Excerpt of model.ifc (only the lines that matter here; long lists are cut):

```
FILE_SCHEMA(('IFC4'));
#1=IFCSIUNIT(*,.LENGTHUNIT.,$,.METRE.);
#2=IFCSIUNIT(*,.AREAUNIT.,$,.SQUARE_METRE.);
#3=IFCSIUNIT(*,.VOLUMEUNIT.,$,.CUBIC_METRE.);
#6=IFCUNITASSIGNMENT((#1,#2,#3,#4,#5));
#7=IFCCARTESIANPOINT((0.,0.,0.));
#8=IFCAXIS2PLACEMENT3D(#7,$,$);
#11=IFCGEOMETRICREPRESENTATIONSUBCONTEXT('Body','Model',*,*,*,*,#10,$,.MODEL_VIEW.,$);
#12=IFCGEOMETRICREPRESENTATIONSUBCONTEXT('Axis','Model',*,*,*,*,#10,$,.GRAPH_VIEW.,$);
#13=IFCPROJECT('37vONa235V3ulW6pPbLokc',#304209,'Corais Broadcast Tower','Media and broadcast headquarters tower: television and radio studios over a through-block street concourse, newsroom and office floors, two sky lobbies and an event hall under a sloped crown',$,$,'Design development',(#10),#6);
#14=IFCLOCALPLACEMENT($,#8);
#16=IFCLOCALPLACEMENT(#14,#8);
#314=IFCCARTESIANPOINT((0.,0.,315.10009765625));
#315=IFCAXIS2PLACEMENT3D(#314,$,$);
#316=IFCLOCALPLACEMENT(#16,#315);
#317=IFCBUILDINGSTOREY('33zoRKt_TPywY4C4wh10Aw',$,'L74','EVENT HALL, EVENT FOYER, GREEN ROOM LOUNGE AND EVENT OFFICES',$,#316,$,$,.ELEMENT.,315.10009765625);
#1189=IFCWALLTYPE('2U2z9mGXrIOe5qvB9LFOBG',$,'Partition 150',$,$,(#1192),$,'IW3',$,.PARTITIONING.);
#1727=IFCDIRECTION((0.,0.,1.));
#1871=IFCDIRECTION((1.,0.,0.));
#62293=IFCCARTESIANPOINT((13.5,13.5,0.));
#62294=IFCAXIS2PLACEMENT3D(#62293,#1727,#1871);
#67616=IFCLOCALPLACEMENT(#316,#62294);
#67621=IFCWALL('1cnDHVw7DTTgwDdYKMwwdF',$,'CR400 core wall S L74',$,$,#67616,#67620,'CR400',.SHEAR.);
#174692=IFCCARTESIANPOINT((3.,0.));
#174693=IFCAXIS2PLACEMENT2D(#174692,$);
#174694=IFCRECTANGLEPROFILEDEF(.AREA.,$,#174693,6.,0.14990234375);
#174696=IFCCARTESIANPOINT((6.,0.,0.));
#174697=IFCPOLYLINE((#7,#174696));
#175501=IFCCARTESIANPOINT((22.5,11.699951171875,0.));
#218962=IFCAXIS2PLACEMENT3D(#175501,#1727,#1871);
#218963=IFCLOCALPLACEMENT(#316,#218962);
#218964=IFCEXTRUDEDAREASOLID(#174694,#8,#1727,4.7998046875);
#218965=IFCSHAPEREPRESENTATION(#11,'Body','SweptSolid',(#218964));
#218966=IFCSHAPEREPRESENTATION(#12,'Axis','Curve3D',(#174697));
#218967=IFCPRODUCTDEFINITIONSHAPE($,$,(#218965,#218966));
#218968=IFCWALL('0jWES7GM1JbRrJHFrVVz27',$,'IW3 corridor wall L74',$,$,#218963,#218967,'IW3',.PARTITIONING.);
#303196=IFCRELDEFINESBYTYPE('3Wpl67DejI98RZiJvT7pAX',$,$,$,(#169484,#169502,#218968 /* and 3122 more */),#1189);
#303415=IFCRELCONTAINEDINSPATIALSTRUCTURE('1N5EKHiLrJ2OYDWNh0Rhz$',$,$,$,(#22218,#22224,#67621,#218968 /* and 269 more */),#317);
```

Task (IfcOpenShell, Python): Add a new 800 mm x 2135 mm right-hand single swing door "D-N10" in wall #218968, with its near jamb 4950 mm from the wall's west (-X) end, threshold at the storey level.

```python
import numpy as np
import ifcopenshell
import ifcopenshell.api.feature
import ifcopenshell.api.geometry
import ifcopenshell.api.root
import ifcopenshell.api.spatial
import ifcopenshell.geom
import ifcopenshell.util.element
import ifcopenshell.util.placement
import ifcopenshell.util.representation
import ifcopenshell.util.shape
import ifcopenshell.util.unit

model = ifcopenshell.open("model.ifc")
unit_scale = ifcopenshell.util.unit.calculate_unit_scale(model)
settings = ifcopenshell.geom.settings()


def volume(element):
    """Net volume in cubic metres, openings subtracted."""
    shape = ifcopenshell.geom.create_shape(settings, element)
    return ifcopenshell.util.shape.get_volume(shape.geometry)


wall = model.by_guid("0jWES7GM1JbRrJHFrVVz27")
storey = ifcopenshell.util.element.get_container(wall, ifc_class="IfcBuildingStorey")
context = ifcopenshell.util.representation.get_context(model, "Model", "Body", "MODEL_VIEW")
before = volume(wall)

width, height, from_end, sill = 0.8, 2.135, 4.95, 0.0  # metres

# The wall runs along its own X axis, and the end named is its -X end.
wall_shape = ifcopenshell.geom.create_shape(settings, wall)
x, y, z = ifcopenshell.util.shape.get_vertices(wall_shape.geometry).T
start = x.min() + from_end
face, thickness = float(y.min()), float(y.max() - y.min())
wall_matrix = ifcopenshell.util.placement.get_local_placement(wall.ObjectPlacement)
level = ifcopenshell.util.placement.get_local_placement(storey.ObjectPlacement)[2, 3]


def in_wall(x, y):
    """Placement at x, y metres in the wall's axes, at sill height."""
    matrix = wall_matrix.copy()
    matrix[:, 3] = wall_matrix @ np.array([x / unit_scale, y / unit_scale, 0.0, 1.0])
    matrix[2, 3] = level + sill / unit_scale
    return matrix


# Opening: a box that overshoots both wall faces by 50 mm.
opening = ifcopenshell.api.root.create_entity(model, ifc_class="IfcOpeningElement", predefined_type="OPENING")
box = ifcopenshell.api.geometry.add_wall_representation(
    model, context=context, length=width, height=height, thickness=thickness + 0.1
)
ifcopenshell.api.geometry.assign_representation(model, product=opening, representation=box)
ifcopenshell.api.geometry.edit_object_placement(model, product=opening, matrix=in_wall(start, face - 0.05), is_si=False)
ifcopenshell.api.feature.add_feature(model, feature=opening, element=wall)

door = ifcopenshell.api.root.create_entity(model, ifc_class="IfcDoor", name="D-N10", predefined_type="DOOR")
door.OverallWidth, door.OverallHeight = width / unit_scale, height / unit_scale
door.OperationType = "SINGLE_SWING_RIGHT"
body = ifcopenshell.api.geometry.add_door_representation(
    model,
    context=context,
    overall_width=door.OverallWidth,
    overall_height=door.OverallHeight,
    operation_type="SINGLE_SWING_RIGHT",
    lining_properties={"LiningDepth": thickness / unit_scale, "ThresholdDepth": thickness / unit_scale},
)
ifcopenshell.api.geometry.assign_representation(model, product=door, representation=body)
ifcopenshell.api.spatial.assign_container(model, products=[door], relating_structure=storey)
ifcopenshell.api.feature.add_filling(model, opening=opening, element=door)

# The lining spans the wall, so the door starts at the wall face.
ifcopenshell.api.geometry.edit_object_placement(model, product=door, matrix=in_wall(start, face), is_si=False)

after = volume(wall)

print(f"wall volume {before:.3f} -> {after:.3f} m3")

model.write("model_updated.ifc")
```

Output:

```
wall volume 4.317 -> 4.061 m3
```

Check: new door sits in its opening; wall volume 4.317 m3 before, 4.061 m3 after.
